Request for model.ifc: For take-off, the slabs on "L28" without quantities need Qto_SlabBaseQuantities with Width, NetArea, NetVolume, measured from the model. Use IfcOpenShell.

First a look at what the model holds.

```python
import ifcopenshell
import ifcopenshell.util.element
import ifcopenshell.util.unit

model = ifcopenshell.open("model.ifc")
print(model.schema)
for unit_type in ("LENGTHUNIT", "AREAUNIT", "VOLUMEUNIT"):
    print(unit_type, ifcopenshell.util.unit.calculate_unit_scale(model, unit_type))
storey = next(s for s in model.by_type("IfcBuildingStorey") if s.Name == "L28")
slabs = [e for e in ifcopenshell.util.element.get_decomposition(storey) if e.is_a("IfcSlab")]
for e in sorted(slabs, key=lambda e: e.id()):
    print(e.id(), e.is_a(), e.Name, list(ifcopenshell.util.element.get_psets(e, qtos_only=True)), sep=" | ")
```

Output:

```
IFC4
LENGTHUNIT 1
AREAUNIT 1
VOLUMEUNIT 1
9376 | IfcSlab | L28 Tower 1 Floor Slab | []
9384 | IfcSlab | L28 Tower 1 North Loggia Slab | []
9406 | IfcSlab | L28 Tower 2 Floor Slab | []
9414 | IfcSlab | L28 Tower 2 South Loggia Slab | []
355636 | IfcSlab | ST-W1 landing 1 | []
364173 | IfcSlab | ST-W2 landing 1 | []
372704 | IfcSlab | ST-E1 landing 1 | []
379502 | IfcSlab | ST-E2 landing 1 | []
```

```python
import ifcopenshell
import ifcopenshell.api.pset
import ifcopenshell.geom
import ifcopenshell.util.element
import ifcopenshell.util.shape
import ifcopenshell.util.unit

model = ifcopenshell.open("model.ifc")
unit_scale = ifcopenshell.util.unit.calculate_unit_scale(model)
area_scale = ifcopenshell.util.unit.calculate_unit_scale(model, "AREAUNIT")
volume_scale = ifcopenshell.util.unit.calculate_unit_scale(model, "VOLUMEUNIT")
settings = ifcopenshell.geom.settings()

storey = next(s for s in model.by_type("IfcBuildingStorey") if s.Name == "L28")
slabs = [e for e in ifcopenshell.util.element.get_decomposition(storey) if e.is_a("IfcSlab")]

for e in sorted(slabs, key=lambda e: e.id()):
    if ifcopenshell.util.element.get_psets(e, qtos_only=True, should_inherit=False):
        continue
    # Geometry comes back in metres, in the element's own axes.
    shape = ifcopenshell.geom.create_shape(settings, e)
    values = {
        "Width": ifcopenshell.util.shape.get_z(shape.geometry) / unit_scale,
        "NetArea": ifcopenshell.util.shape.get_footprint_area(shape.geometry) / area_scale,
        "NetVolume": ifcopenshell.util.shape.get_volume(shape.geometry) / volume_scale,
    }
    qto = ifcopenshell.api.pset.add_qto(model, product=e, name="Qto_SlabBaseQuantities")
    ifcopenshell.api.pset.edit_qto(model, qto=qto, properties=values)
    print(e.id(), {k: round(v, 3) for k, v in values.items()})

model.write("model_v2.ifc")
```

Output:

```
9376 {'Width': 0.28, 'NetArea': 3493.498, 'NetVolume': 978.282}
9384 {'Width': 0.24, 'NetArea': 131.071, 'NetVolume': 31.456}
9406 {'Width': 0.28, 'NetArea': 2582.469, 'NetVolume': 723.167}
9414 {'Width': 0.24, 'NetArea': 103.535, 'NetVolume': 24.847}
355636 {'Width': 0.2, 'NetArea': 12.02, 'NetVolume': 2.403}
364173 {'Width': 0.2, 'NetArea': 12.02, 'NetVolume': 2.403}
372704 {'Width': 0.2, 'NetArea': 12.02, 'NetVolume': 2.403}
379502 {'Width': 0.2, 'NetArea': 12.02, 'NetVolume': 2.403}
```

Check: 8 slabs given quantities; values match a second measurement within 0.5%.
